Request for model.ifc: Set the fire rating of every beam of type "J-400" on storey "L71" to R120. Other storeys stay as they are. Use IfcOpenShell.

First a look at what the model holds.

```python
import ifcopenshell
import ifcopenshell.util.element

model = ifcopenshell.open("model.ifc")
print(model.schema)
storey = next(s for s in model.by_type("IfcBuildingStorey") if s.Name == "L71")
beams = [e for e in ifcopenshell.util.element.get_decomposition(storey) if e.is_a("IfcBeam")]
seen = {}
for e in beams:
    element_type = ifcopenshell.util.element.get_type(e)
    key = (element_type.Name if element_type != e and element_type else None, ifcopenshell.util.element.get_pset(e, "Pset_BeamCommon", "FireRating"))
    seen[key] = seen.get(key, 0) + 1
for (name, value), count in sorted(seen.items(), key=str):
    print(count, "x", name, "|", value)
```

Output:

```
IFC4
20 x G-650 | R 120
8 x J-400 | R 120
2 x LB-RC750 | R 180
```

```python
import ifcopenshell
import ifcopenshell.api.pset
import ifcopenshell.util.element

model = ifcopenshell.open("model.ifc")

storey = next(s for s in model.by_type("IfcBuildingStorey") if s.Name == "L71")
beams = [e for e in ifcopenshell.util.element.get_decomposition(storey) if e.is_a("IfcBeam")]

count = 0
for e in beams:
    element_type = ifcopenshell.util.element.get_type(e)
    if element_type in (None, e) or element_type.Name != "J-400":
        continue
    found = ifcopenshell.util.element.get_pset(e, "Pset_BeamCommon", should_inherit=False)
    if found:
        pset = model.by_id(found["id"])
        if len(ifcopenshell.util.element.get_elements_by_pset(pset)) > 1:
            pset = ifcopenshell.api.pset.unshare_pset(model, products=[e], pset=pset)[0]
    else:
        pset = ifcopenshell.api.pset.add_pset(model, product=e, name="Pset_BeamCommon")
    ifcopenshell.api.pset.edit_pset(model, pset=pset, properties={"FireRating": "R120"})
    count += 1

print(count, "beams updated")

model.write("model_v2.ifc")
```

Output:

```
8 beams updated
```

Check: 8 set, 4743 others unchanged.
